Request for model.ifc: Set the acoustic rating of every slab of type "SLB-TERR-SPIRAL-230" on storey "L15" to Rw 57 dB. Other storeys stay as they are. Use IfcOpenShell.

First a look at what the model holds.

```python
import ifcopenshell
import ifcopenshell.util.element

model = ifcopenshell.open("model.ifc")
print(model.schema)
storey = next(s for s in model.by_type("IfcBuildingStorey") if s.Name == "L15")
slabs = [e for e in ifcopenshell.util.element.get_decomposition(storey) if e.is_a("IfcSlab")]
seen = {}
for e in slabs:
    element_type = ifcopenshell.util.element.get_type(e)
    key = (element_type.Name if element_type != e and element_type else None, ifcopenshell.util.element.get_pset(e, "Pset_SlabCommon", "AcousticRating"))
    seen[key] = seen.get(key, 0) + 1
for (name, value), count in sorted(seen.items(), key=str):
    print(count, "x", name, "|", value)
```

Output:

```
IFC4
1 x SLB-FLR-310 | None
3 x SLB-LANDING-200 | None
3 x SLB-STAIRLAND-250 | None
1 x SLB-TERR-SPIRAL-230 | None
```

```python
import ifcopenshell
import ifcopenshell.api.pset
import ifcopenshell.util.element

model = ifcopenshell.open("model.ifc")

storey = next(s for s in model.by_type("IfcBuildingStorey") if s.Name == "L15")
slabs = [e for e in ifcopenshell.util.element.get_decomposition(storey) if e.is_a("IfcSlab")]

count = 0
for e in slabs:
    element_type = ifcopenshell.util.element.get_type(e)
    if element_type in (None, e) or element_type.Name != "SLB-TERR-SPIRAL-230":
        continue
    # add_pset returns the element's existing set when there is one.
    pset = ifcopenshell.api.pset.add_pset(model, product=e, name="Pset_SlabCommon")
    ifcopenshell.api.pset.edit_pset(model, pset=pset, properties={"AcousticRating": "Rw 57 dB"})
    count += 1

print(count, "slabs updated")

model.write("model_updated.ifc")
```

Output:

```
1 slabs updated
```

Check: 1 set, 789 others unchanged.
